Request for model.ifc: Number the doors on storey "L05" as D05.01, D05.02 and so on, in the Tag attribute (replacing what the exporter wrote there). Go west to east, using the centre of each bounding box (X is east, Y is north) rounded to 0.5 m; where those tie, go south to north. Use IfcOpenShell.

First a look at what the model holds.

```python
import ifcopenshell
import ifcopenshell.util.element
import ifcopenshell.util.placement

model = ifcopenshell.open("model.ifc")
print(model.schema)
storey = next(s for s in model.by_type("IfcBuildingStorey") if s.Name == "L05")
doors = [e for e in ifcopenshell.util.element.get_decomposition(storey) if e.is_a("IfcDoor")]
for e in sorted(doors, key=lambda e: e.id()):
    origin = ifcopenshell.util.placement.get_local_placement(e.ObjectPlacement)[:3, 3]
    print(e.id(), e.Tag, e.Name, origin.round(2) + 0.0, sep=" | ")
```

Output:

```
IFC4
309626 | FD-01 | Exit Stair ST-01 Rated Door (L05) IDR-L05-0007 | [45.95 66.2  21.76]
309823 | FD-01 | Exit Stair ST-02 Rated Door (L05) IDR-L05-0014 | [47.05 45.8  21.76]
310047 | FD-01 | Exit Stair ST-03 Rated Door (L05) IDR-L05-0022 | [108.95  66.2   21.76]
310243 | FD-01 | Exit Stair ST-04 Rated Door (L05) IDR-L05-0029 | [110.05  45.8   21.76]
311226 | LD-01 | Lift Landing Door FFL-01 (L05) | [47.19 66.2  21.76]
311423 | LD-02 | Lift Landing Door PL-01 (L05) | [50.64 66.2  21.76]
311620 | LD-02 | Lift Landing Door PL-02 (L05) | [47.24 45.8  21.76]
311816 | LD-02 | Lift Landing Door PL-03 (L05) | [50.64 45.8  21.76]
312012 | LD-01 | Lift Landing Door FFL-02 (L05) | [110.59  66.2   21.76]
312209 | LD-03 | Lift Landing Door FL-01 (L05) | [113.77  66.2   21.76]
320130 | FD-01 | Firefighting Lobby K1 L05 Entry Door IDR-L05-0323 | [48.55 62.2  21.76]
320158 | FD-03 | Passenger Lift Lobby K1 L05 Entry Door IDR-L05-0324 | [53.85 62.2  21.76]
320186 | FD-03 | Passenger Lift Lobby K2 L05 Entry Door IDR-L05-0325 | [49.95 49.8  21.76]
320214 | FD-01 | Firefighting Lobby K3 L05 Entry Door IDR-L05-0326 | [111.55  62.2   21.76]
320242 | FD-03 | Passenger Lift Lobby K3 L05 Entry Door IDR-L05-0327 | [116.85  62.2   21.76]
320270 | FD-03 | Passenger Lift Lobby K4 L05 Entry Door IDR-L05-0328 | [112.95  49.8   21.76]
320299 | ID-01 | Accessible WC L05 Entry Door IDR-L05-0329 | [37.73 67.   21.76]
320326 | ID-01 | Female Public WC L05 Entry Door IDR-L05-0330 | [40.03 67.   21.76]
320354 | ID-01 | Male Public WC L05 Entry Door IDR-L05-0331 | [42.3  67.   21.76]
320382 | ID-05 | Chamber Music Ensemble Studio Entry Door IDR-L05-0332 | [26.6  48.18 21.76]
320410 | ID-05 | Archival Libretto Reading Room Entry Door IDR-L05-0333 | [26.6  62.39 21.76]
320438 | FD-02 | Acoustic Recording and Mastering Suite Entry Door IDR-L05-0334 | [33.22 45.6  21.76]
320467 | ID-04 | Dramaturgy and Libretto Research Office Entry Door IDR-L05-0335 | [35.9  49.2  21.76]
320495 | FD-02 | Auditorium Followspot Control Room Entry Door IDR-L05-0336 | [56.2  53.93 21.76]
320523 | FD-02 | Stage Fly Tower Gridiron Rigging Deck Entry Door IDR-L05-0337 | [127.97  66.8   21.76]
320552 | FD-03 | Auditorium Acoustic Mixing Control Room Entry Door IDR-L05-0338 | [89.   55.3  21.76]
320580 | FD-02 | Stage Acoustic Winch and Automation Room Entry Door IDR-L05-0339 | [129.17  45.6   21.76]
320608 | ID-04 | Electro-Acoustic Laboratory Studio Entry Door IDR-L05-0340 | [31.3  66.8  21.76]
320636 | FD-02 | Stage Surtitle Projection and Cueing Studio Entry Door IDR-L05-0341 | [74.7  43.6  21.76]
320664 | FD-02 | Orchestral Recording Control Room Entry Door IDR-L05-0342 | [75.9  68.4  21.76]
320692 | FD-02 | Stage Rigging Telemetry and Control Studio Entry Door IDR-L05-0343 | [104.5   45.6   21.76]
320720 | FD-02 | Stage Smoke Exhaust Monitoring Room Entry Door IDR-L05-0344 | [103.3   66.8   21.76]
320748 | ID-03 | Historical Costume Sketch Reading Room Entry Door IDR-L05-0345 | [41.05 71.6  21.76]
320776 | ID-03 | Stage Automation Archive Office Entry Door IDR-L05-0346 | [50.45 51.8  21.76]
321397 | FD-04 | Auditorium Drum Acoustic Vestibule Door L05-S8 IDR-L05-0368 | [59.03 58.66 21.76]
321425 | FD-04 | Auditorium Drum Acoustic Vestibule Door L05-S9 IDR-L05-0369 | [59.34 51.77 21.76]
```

```python
import ifcopenshell
import ifcopenshell.geom
import ifcopenshell.util.element
import ifcopenshell.util.shape

model = ifcopenshell.open("model.ifc")
settings = ifcopenshell.geom.settings()
settings.set("use-world-coords", True)


def centre(element):
    shape = ifcopenshell.geom.create_shape(settings, element)
    return ifcopenshell.util.shape.get_bbox_centroid(shape.geometry)


storey = next(s for s in model.by_type("IfcBuildingStorey") if s.Name == "L05")
doors = [e for e in ifcopenshell.util.element.get_decomposition(storey) if e.is_a("IfcDoor")]

# Insertion points can sit at a corner or the storey origin, so sort by the geometry (in metres).
centres = {e: centre(e) for e in doors}
doors.sort(key=lambda e: (round(centres[e][0] / 0.5), centres[e][1]))

for i, e in enumerate(doors, start=1):
    number = f"D05.{i:02d}"
    e.Tag = number
    print(e.id(), number)

model.write("model-out.ifc")
```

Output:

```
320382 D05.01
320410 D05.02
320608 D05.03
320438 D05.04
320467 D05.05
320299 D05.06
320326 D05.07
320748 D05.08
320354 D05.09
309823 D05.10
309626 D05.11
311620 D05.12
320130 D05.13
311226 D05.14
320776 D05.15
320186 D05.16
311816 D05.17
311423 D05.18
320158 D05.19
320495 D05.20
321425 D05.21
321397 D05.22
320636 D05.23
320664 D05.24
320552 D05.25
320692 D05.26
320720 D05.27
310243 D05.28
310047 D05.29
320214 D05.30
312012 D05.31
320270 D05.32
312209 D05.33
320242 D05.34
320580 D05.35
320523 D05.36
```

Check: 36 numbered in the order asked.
